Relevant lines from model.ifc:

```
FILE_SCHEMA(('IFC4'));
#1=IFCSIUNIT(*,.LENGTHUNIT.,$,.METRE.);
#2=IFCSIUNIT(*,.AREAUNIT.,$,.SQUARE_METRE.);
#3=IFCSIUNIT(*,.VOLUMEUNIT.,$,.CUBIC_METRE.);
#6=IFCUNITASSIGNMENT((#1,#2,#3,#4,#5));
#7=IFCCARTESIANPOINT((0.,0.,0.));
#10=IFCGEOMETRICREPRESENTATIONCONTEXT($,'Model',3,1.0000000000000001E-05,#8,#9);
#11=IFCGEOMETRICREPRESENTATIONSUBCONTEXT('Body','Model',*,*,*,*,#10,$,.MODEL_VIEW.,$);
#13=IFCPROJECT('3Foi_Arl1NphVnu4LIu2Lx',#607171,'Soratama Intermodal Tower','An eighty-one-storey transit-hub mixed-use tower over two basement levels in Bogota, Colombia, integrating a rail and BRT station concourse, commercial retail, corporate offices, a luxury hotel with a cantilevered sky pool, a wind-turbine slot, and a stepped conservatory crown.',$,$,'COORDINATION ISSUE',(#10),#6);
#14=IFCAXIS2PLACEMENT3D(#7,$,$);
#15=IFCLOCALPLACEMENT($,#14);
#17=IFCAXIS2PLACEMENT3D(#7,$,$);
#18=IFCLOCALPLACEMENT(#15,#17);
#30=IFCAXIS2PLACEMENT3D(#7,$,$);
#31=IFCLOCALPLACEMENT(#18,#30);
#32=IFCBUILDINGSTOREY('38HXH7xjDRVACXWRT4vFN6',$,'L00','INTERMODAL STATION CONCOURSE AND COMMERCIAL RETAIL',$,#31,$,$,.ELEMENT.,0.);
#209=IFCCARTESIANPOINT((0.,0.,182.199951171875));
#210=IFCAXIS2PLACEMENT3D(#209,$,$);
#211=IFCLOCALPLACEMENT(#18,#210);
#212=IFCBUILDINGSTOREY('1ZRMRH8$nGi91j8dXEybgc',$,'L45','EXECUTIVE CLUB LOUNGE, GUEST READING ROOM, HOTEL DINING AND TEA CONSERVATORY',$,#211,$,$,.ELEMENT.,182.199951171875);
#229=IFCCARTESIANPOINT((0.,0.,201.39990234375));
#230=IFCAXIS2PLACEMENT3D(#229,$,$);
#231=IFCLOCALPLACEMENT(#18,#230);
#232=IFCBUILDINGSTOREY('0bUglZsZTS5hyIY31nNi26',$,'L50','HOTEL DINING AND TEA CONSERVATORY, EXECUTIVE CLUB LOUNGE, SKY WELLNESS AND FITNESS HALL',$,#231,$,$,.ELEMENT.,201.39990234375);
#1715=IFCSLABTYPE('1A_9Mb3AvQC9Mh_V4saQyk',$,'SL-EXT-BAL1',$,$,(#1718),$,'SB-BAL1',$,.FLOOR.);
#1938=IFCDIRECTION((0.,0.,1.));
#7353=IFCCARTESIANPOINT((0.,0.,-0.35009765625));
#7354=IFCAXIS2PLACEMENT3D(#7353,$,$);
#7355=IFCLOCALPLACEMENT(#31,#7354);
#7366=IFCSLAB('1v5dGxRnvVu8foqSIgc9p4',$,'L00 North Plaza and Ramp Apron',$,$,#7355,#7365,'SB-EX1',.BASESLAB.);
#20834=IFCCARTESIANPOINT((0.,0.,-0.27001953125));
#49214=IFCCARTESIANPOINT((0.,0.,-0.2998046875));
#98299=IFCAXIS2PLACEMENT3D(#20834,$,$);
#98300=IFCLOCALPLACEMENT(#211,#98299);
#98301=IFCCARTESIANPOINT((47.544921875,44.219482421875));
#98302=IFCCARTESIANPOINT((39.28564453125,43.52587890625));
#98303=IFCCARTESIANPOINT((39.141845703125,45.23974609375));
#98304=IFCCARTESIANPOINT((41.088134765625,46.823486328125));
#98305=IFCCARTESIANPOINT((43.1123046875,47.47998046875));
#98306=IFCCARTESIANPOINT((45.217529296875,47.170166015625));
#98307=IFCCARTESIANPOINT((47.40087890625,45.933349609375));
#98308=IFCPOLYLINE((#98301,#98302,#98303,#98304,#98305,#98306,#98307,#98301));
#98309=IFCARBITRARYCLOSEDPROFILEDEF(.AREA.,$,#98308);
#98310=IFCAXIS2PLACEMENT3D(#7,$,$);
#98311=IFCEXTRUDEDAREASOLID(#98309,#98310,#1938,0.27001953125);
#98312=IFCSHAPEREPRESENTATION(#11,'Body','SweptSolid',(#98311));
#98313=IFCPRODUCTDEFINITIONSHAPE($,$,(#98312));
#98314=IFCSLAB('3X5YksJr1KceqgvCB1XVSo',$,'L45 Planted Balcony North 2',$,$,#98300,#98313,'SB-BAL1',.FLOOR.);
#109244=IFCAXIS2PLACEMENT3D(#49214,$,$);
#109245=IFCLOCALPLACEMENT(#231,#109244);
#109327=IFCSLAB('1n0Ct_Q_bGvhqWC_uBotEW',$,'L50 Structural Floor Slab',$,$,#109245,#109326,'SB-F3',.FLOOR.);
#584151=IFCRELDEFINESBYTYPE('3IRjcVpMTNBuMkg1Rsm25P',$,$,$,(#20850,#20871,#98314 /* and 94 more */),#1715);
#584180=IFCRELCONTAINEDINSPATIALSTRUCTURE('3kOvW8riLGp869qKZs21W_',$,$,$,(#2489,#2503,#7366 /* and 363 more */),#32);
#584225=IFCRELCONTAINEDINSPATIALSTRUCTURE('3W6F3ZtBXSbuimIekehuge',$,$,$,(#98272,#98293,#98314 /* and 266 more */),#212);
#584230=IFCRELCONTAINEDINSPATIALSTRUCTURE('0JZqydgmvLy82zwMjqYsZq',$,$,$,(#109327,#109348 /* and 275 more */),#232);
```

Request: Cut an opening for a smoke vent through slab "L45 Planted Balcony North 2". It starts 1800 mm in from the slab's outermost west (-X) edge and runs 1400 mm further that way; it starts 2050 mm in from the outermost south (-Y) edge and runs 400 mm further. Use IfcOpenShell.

```python
import numpy as np
import ifcopenshell
import ifcopenshell.api.feature
import ifcopenshell.api.geometry
import ifcopenshell.api.root
import ifcopenshell.geom
import ifcopenshell.util.placement
import ifcopenshell.util.representation
import ifcopenshell.util.shape
import ifcopenshell.util.unit

model = ifcopenshell.open("model.ifc")
unit_scale = ifcopenshell.util.unit.calculate_unit_scale(model)
settings = ifcopenshell.geom.settings()


def volume(element):
    """Net volume in cubic metres, openings subtracted."""
    shape = ifcopenshell.geom.create_shape(settings, element)
    return ifcopenshell.util.shape.get_volume(shape.geometry)


slab = model.by_guid("3X5YksJr1KceqgvCB1XVSo")
before = volume(slab)

# Extent in the slab's own axes, in metres. The edges named are its -X and -Y sides.
slab_shape = ifcopenshell.geom.create_shape(settings, slab)
vertices = ifcopenshell.util.shape.get_vertices(slab_shape.geometry)
x_min, y_min, bottom = vertices.min(axis=0)
top = vertices[:, 2].max()

opening = ifcopenshell.api.root.create_entity(model, ifc_class="IfcOpeningElement", name="Smoke vent opening", predefined_type="OPENING")
context = ifcopenshell.util.representation.get_context(model, "Model", "Body", "MODEL_VIEW")
width, depth = 1.4, 0.4
outline = [(0.0, 0.0), (width, 0.0), (width, depth), (0.0, depth), (0.0, 0.0)]
# Overshoot both faces by 50 mm so the cut is clean.
shape = ifcopenshell.api.geometry.add_slab_representation(
    model, context=context, depth=top - bottom + 0.1, polyline=outline
)
ifcopenshell.api.geometry.assign_representation(model, product=opening, representation=shape)

matrix = ifcopenshell.util.placement.get_local_placement(slab.ObjectPlacement)
matrix[:, 3] = matrix @ np.append(np.array([x_min + 1.8, y_min + 2.05, bottom - 0.05]) / unit_scale, 1.0)
ifcopenshell.api.geometry.edit_object_placement(model, product=opening, matrix=matrix, is_si=False)
ifcopenshell.api.feature.add_feature(model, feature=opening, element=slab)

after = volume(slab)

print(f"slab volume {before:.3f} -> {after:.3f} m3")

model.write("model-out.ifc")
```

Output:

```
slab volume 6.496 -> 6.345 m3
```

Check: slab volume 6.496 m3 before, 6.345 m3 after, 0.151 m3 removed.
